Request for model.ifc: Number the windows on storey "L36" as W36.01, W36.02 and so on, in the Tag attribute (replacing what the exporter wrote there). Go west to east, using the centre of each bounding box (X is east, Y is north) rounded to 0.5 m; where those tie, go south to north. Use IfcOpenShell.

First a look at what the model holds.

```python
import ifcopenshell
import ifcopenshell.util.element
import ifcopenshell.util.placement

model = ifcopenshell.open("model.ifc")
print(model.schema)
storey = next(s for s in model.by_type("IfcBuildingStorey") if s.Name == "L36")
windows = [e for e in ifcopenshell.util.element.get_decomposition(storey) if e.is_a("IfcWindow")]
for e in sorted(windows, key=lambda e: e.id()):
    origin = ifcopenshell.util.placement.get_local_placement(e.ObjectPlacement)[:3, 3]
    print(e.id(), e.Tag, e.Name, origin.round(2) + 0.0, sep=" | ")
```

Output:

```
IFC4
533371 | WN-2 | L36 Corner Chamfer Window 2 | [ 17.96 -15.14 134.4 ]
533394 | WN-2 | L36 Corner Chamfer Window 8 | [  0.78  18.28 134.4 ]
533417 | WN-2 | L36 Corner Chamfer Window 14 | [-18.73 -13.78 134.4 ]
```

```python
import ifcopenshell
import ifcopenshell.geom
import ifcopenshell.util.element
import ifcopenshell.util.shape

model = ifcopenshell.open("model.ifc")
settings = ifcopenshell.geom.settings()
settings.set("use-world-coords", True)


def centre(element):
    shape = ifcopenshell.geom.create_shape(settings, element)
    return ifcopenshell.util.shape.get_bbox_centroid(shape.geometry)


storey = next(s for s in model.by_type("IfcBuildingStorey") if s.Name == "L36")
windows = [e for e in ifcopenshell.util.element.get_decomposition(storey) if e.is_a("IfcWindow")]

# Insertion points can sit at a corner or the storey origin, so sort by the geometry (in metres).
centres = {e: centre(e) for e in windows}
windows.sort(key=lambda e: (round(centres[e][0] / 0.5), centres[e][1]))

for i, e in enumerate(windows, start=1):
    number = f"W36.{i:02d}"
    e.Tag = number
    print(e.id(), number)

model.write("model_v2.ifc")
```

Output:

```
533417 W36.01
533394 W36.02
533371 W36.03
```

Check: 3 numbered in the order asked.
